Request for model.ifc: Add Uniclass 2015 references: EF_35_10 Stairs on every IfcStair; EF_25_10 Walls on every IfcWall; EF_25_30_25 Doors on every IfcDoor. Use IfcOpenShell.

First a look at what the model holds.

```python
import ifcopenshell

model = ifcopenshell.open("model.ifc")
print(model.schema)
print("classifications:", [c.Name for c in model.by_type("IfcClassification")])
for ifc_class in ("IfcDoor", "IfcRoof", "IfcStair", "IfcWall", "IfcWindow"):
    print(ifc_class, len(model.by_type(ifc_class)))
```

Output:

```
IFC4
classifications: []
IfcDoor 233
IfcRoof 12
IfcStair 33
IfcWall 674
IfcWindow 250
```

```python
import ifcopenshell
import ifcopenshell.api.classification

model = ifcopenshell.open("model.ifc")

system = ifcopenshell.api.classification.add_classification(model, classification="Uniclass 2015")

codes = {
    "IfcStair": ("EF_35_10", "Stairs"),
    "IfcWall": ("EF_25_10", "Walls"),
    "IfcDoor": ("EF_25_30_25", "Doors"),
}
for ifc_class, (code, name) in codes.items():
    products = model.by_type(ifc_class)
    ifcopenshell.api.classification.add_reference(
        model, products=products, classification=system, identification=code, name=name
    )
    print(code, len(products))

model.write("model_edited.ifc")
```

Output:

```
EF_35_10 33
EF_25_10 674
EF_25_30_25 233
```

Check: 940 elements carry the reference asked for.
